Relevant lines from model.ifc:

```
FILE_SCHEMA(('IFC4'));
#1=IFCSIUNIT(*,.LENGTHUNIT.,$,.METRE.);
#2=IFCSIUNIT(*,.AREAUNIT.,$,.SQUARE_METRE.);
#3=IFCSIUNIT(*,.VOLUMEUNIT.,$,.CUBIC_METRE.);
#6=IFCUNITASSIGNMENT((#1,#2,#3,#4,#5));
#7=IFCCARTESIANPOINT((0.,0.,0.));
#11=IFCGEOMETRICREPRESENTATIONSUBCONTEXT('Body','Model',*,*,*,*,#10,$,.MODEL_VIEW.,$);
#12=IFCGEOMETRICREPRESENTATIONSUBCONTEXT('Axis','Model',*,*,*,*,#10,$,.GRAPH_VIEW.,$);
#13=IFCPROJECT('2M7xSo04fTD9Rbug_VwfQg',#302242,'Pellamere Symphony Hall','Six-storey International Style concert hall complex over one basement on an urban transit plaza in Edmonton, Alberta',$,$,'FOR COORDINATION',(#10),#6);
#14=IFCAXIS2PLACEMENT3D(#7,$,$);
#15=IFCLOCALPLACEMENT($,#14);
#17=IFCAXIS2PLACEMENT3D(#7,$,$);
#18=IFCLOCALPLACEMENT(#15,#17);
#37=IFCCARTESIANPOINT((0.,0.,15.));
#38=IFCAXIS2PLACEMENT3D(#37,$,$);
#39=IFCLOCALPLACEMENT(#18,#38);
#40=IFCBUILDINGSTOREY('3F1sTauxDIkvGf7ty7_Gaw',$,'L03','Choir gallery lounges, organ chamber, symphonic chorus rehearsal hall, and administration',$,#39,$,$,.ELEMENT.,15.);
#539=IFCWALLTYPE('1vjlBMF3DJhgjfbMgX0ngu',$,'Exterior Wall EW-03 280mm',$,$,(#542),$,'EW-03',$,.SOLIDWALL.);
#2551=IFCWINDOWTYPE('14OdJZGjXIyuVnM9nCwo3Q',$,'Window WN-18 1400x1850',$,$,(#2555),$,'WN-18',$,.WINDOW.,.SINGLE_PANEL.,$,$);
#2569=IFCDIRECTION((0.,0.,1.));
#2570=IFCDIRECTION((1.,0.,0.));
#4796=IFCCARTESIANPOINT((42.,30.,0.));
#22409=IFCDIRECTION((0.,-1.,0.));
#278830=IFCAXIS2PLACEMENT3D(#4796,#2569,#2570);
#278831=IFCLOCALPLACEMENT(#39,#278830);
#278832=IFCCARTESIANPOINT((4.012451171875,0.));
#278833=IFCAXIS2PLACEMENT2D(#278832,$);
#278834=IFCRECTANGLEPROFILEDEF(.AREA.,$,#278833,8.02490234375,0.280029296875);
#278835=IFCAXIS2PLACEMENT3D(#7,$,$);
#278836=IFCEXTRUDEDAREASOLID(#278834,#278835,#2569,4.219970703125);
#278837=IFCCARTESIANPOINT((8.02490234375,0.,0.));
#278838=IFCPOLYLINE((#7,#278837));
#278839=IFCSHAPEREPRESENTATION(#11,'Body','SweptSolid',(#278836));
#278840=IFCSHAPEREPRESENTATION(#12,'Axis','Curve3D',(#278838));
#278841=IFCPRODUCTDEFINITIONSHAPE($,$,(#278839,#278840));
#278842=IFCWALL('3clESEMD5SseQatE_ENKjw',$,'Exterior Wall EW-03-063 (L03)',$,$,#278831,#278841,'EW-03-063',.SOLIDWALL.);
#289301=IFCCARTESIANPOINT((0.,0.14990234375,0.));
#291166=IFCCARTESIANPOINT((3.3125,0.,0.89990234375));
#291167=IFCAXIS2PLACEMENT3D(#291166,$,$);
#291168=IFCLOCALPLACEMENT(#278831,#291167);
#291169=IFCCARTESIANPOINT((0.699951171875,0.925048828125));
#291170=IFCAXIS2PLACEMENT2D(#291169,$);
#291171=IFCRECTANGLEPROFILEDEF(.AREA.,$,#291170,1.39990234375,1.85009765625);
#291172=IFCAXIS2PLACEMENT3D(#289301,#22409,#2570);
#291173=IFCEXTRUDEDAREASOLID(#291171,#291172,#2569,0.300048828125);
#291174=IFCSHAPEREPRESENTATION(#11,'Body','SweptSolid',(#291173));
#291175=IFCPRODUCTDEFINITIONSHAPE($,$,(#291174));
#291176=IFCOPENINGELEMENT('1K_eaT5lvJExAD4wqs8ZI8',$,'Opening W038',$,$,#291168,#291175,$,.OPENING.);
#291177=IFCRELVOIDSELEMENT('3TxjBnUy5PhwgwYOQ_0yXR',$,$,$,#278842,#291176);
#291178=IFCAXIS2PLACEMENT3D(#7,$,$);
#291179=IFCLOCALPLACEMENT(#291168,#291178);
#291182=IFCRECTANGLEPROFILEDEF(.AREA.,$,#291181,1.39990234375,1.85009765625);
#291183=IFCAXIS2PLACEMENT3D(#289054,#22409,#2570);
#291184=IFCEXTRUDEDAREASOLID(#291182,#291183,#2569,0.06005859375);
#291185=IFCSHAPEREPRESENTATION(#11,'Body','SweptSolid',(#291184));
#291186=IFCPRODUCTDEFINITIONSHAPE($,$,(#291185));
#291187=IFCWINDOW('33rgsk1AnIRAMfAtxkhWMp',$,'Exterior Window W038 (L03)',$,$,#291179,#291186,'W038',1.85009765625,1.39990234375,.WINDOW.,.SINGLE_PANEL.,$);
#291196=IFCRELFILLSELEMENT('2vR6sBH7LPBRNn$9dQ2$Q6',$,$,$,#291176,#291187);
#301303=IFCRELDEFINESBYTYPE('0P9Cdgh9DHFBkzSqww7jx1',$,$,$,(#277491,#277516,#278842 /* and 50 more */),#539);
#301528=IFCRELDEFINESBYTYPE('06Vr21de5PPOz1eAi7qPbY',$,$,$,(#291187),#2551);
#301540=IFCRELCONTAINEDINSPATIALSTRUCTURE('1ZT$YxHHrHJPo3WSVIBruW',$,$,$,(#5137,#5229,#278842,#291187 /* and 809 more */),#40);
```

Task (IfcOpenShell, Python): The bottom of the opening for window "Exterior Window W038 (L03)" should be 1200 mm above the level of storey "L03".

```python
import numpy as np
import ifcopenshell
import ifcopenshell.api.geometry
import ifcopenshell.geom
import ifcopenshell.util.element
import ifcopenshell.util.placement
import ifcopenshell.util.shape
import ifcopenshell.util.unit

model = ifcopenshell.open("model.ifc")
unit_scale = ifcopenshell.util.unit.calculate_unit_scale(model)

window = model.by_guid("33rgsk1AnIRAMfAtxkhWMp")
opening = window.FillsVoids[0].RelatingOpeningElement
storey = ifcopenshell.util.element.get_container(window, ifc_class="IfcBuildingStorey")
level = ifcopenshell.util.placement.get_local_placement(storey.ObjectPlacement)[2, 3]

# The opening's origin need not be at the sill, so measure its lowest point.
shape = ifcopenshell.geom.create_shape(ifcopenshell.geom.settings(), opening)
bottom = ifcopenshell.util.shape.get_shape_bottom_elevation(shape, shape.geometry) / unit_scale
dz = level + 1.2 - bottom

shift = np.array([0.0, 0.0, dz])
# The window is placed relative to its opening, so it follows when the opening moves.
matrix = ifcopenshell.util.placement.get_local_placement(opening.ObjectPlacement)
matrix[:3, 3] += shift
ifcopenshell.api.geometry.edit_object_placement(
    model, product=opening, matrix=matrix, is_si=False, should_transform_children=True
)

print(f"moved by {dz * unit_scale:+.3f} m")

model.write("model-out.ifc")
```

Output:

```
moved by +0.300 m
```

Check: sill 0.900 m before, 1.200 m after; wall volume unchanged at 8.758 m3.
